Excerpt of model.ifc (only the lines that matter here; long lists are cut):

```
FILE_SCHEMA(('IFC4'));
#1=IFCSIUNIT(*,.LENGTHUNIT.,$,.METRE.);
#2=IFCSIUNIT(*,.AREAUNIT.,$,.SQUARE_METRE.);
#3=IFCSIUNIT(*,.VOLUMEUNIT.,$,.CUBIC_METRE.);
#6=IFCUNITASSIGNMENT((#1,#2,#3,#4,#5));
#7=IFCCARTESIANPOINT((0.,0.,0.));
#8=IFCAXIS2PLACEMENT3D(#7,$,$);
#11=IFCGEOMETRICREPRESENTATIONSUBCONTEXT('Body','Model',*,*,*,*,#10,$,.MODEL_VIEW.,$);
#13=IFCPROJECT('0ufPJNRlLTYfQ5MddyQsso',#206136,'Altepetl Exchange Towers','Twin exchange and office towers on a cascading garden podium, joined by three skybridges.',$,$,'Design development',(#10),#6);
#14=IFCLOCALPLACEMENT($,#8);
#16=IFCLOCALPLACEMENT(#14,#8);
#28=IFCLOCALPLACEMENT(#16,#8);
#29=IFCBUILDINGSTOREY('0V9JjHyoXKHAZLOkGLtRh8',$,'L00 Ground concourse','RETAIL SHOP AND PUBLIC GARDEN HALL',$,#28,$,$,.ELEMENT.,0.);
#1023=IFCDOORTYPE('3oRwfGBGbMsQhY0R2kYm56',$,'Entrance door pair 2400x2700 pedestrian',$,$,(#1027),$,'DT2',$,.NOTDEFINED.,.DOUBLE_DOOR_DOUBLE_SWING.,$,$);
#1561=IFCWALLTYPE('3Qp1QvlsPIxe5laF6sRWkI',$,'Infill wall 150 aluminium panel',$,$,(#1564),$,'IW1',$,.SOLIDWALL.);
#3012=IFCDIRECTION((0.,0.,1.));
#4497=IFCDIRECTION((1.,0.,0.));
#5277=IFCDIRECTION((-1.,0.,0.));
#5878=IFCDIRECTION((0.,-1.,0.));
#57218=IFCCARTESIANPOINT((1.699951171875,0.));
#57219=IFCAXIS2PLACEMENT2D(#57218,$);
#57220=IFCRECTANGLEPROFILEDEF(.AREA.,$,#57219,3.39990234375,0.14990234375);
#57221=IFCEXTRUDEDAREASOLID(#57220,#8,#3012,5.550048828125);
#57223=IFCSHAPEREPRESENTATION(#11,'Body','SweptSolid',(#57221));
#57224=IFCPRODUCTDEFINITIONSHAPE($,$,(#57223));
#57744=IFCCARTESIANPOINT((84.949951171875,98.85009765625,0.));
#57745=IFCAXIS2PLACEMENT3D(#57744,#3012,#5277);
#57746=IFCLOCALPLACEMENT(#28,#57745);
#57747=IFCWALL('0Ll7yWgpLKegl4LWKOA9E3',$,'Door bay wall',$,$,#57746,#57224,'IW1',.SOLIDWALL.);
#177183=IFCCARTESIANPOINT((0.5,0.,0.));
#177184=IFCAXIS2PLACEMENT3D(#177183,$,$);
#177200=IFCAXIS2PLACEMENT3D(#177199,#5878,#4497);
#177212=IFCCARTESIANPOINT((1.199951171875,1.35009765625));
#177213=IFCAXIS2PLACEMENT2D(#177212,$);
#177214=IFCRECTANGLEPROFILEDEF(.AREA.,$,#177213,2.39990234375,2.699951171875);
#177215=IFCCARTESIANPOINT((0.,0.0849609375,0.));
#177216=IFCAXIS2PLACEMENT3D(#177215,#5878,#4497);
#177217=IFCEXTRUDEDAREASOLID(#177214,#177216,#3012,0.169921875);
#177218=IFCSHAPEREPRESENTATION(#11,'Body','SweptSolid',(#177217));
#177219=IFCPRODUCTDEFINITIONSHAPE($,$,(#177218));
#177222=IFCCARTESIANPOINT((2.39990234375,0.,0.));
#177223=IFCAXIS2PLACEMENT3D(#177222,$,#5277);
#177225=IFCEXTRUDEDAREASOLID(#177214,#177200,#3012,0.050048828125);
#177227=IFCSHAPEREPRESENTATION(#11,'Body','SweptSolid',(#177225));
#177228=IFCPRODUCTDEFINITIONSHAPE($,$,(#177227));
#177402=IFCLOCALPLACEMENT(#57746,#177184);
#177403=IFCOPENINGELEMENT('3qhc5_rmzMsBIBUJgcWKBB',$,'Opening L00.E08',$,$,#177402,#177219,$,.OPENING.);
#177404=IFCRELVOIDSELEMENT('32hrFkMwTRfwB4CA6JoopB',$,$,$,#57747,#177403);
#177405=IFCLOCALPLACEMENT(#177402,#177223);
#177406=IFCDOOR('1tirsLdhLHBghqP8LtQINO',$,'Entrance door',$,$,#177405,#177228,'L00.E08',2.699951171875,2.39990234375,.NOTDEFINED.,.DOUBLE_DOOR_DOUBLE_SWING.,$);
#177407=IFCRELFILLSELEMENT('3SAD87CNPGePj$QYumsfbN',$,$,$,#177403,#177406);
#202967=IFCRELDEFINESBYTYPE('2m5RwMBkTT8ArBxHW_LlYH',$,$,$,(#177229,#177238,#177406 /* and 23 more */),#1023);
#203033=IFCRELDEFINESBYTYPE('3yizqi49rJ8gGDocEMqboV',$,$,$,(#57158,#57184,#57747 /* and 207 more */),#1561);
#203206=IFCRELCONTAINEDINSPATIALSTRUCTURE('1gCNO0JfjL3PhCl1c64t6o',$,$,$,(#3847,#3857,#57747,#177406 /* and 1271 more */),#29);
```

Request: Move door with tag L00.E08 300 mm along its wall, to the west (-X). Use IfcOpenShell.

```python
import ifcopenshell
import ifcopenshell.api.geometry
import ifcopenshell.util.placement
import ifcopenshell.util.unit

model = ifcopenshell.open("model.ifc")
unit_scale = ifcopenshell.util.unit.calculate_unit_scale(model)

door = model.by_guid("1tirsLdhLHBghqP8LtQINO")
opening = door.FillsVoids[0].RelatingOpeningElement
wall = opening.VoidsElements[0].RelatingBuildingElement

wall_matrix = ifcopenshell.util.placement.get_local_placement(wall.ObjectPlacement)
shift = wall_matrix[:3, 0] * 0.3 / unit_scale
before = ifcopenshell.util.placement.get_local_placement(door.ObjectPlacement)[:3, 3].copy()

# The door is placed relative to its opening, so it follows when the opening moves.
matrix = ifcopenshell.util.placement.get_local_placement(opening.ObjectPlacement)
matrix[:3, 3] += shift
ifcopenshell.api.geometry.edit_object_placement(
    model, product=opening, matrix=matrix, is_si=False, should_transform_children=True
)

after = ifcopenshell.util.placement.get_local_placement(door.ObjectPlacement)[:3, 3]
print("door moved by", (after - before).round(3) + 0.0)

model.write("model_rev.ifc")
```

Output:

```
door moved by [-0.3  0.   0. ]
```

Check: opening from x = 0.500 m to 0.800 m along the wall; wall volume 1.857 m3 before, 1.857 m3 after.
